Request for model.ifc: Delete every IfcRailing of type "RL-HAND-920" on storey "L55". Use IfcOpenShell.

First a look at what the model holds.

```python
import ifcopenshell
import ifcopenshell.util.element

model = ifcopenshell.open("model.ifc")
print(model.schema)
storey = next(s for s in model.by_type("IfcBuildingStorey") if s.Name == "L55")
railings = [e for e in ifcopenshell.util.element.get_decomposition(storey) if e.is_a("IfcRailing")]
seen = {}
for e in railings:
    element_type = ifcopenshell.util.element.get_type(e)
    name = element_type.Name if element_type not in (None, e) else None
    seen[name] = seen.get(name, 0) + 1
for name, count in sorted(seen.items(), key=str):
    print(count, "x", name)
```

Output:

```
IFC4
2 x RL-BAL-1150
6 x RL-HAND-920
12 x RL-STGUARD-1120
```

```python
import ifcopenshell
import ifcopenshell.api.root
import ifcopenshell.util.element

model = ifcopenshell.open("model.ifc")

storey = next(s for s in model.by_type("IfcBuildingStorey") if s.Name == "L55")
railings = [e for e in ifcopenshell.util.element.get_decomposition(storey) if e.is_a("IfcRailing")]
targets = [e for e in railings if (t := ifcopenshell.util.element.get_type(e)) not in (None, e) and t.Name == "RL-HAND-920"]

for e in targets:
    ifcopenshell.api.root.remove_product(model, product=e)
print(len(targets), "removed")

model.write("model_v2.ifc")
```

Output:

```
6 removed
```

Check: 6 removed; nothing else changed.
